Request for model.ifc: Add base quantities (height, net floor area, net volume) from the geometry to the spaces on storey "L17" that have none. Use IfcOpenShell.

First a look at what the model holds.

```python
import ifcopenshell
import ifcopenshell.util.element
import ifcopenshell.util.unit

model = ifcopenshell.open("model.ifc")
print(model.schema)
for unit_type in ("LENGTHUNIT", "AREAUNIT", "VOLUMEUNIT"):
    print(unit_type, ifcopenshell.util.unit.calculate_unit_scale(model, unit_type))
storey = next(s for s in model.by_type("IfcBuildingStorey") if s.Name == "L17")
spaces = [e for e in ifcopenshell.util.element.get_decomposition(storey) if e.is_a("IfcSpace")]
for e in sorted(spaces, key=lambda e: e.id()):
    print(e.id(), e.is_a(), e.Name, list(ifcopenshell.util.element.get_psets(e, qtos_only=True)), sep=" | ")
```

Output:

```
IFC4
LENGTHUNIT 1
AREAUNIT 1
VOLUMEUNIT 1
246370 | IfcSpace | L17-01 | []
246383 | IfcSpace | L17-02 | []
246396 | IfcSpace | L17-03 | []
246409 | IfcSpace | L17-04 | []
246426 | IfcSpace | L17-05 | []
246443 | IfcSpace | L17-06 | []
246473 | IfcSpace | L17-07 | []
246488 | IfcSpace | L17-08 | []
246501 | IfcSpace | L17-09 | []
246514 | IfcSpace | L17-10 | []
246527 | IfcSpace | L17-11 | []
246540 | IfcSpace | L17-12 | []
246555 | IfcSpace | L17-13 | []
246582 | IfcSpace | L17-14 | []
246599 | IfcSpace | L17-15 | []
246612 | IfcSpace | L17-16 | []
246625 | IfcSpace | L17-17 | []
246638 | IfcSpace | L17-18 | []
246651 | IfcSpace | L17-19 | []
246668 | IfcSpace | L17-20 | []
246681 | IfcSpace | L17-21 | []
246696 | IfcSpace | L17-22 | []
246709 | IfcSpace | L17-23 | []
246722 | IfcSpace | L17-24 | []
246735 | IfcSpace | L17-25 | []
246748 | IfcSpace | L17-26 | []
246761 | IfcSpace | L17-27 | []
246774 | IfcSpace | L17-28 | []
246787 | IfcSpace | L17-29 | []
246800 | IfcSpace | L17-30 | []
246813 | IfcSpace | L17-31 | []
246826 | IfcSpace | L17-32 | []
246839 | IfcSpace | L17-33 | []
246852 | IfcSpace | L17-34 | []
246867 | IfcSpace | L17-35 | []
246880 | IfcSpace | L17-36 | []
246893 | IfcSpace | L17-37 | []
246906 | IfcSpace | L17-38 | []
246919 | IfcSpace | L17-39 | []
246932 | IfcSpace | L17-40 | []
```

```python
import ifcopenshell
import ifcopenshell.api.pset
import ifcopenshell.geom
import ifcopenshell.util.element
import ifcopenshell.util.shape
import ifcopenshell.util.unit

model = ifcopenshell.open("model.ifc")
unit_scale = ifcopenshell.util.unit.calculate_unit_scale(model)
area_scale = ifcopenshell.util.unit.calculate_unit_scale(model, "AREAUNIT")
volume_scale = ifcopenshell.util.unit.calculate_unit_scale(model, "VOLUMEUNIT")
settings = ifcopenshell.geom.settings()

storey = next(s for s in model.by_type("IfcBuildingStorey") if s.Name == "L17")
spaces = [e for e in ifcopenshell.util.element.get_decomposition(storey) if e.is_a("IfcSpace")]

for e in sorted(spaces, key=lambda e: e.id()):
    if ifcopenshell.util.element.get_psets(e, qtos_only=True, should_inherit=False):
        continue
    # Geometry comes back in metres, in the element's own axes.
    shape = ifcopenshell.geom.create_shape(settings, e)
    values = {
        "Height": ifcopenshell.util.shape.get_z(shape.geometry) / unit_scale,
        "NetFloorArea": ifcopenshell.util.shape.get_footprint_area(shape.geometry) / area_scale,
        "NetVolume": ifcopenshell.util.shape.get_volume(shape.geometry) / volume_scale,
    }
    qto = ifcopenshell.api.pset.add_qto(model, product=e, name="Qto_SpaceBaseQuantities")
    ifcopenshell.api.pset.edit_qto(model, qto=qto, properties=values)
    print(e.id(), {k: round(v, 3) for k, v in values.items()})

model.write("model_edited.ifc")
```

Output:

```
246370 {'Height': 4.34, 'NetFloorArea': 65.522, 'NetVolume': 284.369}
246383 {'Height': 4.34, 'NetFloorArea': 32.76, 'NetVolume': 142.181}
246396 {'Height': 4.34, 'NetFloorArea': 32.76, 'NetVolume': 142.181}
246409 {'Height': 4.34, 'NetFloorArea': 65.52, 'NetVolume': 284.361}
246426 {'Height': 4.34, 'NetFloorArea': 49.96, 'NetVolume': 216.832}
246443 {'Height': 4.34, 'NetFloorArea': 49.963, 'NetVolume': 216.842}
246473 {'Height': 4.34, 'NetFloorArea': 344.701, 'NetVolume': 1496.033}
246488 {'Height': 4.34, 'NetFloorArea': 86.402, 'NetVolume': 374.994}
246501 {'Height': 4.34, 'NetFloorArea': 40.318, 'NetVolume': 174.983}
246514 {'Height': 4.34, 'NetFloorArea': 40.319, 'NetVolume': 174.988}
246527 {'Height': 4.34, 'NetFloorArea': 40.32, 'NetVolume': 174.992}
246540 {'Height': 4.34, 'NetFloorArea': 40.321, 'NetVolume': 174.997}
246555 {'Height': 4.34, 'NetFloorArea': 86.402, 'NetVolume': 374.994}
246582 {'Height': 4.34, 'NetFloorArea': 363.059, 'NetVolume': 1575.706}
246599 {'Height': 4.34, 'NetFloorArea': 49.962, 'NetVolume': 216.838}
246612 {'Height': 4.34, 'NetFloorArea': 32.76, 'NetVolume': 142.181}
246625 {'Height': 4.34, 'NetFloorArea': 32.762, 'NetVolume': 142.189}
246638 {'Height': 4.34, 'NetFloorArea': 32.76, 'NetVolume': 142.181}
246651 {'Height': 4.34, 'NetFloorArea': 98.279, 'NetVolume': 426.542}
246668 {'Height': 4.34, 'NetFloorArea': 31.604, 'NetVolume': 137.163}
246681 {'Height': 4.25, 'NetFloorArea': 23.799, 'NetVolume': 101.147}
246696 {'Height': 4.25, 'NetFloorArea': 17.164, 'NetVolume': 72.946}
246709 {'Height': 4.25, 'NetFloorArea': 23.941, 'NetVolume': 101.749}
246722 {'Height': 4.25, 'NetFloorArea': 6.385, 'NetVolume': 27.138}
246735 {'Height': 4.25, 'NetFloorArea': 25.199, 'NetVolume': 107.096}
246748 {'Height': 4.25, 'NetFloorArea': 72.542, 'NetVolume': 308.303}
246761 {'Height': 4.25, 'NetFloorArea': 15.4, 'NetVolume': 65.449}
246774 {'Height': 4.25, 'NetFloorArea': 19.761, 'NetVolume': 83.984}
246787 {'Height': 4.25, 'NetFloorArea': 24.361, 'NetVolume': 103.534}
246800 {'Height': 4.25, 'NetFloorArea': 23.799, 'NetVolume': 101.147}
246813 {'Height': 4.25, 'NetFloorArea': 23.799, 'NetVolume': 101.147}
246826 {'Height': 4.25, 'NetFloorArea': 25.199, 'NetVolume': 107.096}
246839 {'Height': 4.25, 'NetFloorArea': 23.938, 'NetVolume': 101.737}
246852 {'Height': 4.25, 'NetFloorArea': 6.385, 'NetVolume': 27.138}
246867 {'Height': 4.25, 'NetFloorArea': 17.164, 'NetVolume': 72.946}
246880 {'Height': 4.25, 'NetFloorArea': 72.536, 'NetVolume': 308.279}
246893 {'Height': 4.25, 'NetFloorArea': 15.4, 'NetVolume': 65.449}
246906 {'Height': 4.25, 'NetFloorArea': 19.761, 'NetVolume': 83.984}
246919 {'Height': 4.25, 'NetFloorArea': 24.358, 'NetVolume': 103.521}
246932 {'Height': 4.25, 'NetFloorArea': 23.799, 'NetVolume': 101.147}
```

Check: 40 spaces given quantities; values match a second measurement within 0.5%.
